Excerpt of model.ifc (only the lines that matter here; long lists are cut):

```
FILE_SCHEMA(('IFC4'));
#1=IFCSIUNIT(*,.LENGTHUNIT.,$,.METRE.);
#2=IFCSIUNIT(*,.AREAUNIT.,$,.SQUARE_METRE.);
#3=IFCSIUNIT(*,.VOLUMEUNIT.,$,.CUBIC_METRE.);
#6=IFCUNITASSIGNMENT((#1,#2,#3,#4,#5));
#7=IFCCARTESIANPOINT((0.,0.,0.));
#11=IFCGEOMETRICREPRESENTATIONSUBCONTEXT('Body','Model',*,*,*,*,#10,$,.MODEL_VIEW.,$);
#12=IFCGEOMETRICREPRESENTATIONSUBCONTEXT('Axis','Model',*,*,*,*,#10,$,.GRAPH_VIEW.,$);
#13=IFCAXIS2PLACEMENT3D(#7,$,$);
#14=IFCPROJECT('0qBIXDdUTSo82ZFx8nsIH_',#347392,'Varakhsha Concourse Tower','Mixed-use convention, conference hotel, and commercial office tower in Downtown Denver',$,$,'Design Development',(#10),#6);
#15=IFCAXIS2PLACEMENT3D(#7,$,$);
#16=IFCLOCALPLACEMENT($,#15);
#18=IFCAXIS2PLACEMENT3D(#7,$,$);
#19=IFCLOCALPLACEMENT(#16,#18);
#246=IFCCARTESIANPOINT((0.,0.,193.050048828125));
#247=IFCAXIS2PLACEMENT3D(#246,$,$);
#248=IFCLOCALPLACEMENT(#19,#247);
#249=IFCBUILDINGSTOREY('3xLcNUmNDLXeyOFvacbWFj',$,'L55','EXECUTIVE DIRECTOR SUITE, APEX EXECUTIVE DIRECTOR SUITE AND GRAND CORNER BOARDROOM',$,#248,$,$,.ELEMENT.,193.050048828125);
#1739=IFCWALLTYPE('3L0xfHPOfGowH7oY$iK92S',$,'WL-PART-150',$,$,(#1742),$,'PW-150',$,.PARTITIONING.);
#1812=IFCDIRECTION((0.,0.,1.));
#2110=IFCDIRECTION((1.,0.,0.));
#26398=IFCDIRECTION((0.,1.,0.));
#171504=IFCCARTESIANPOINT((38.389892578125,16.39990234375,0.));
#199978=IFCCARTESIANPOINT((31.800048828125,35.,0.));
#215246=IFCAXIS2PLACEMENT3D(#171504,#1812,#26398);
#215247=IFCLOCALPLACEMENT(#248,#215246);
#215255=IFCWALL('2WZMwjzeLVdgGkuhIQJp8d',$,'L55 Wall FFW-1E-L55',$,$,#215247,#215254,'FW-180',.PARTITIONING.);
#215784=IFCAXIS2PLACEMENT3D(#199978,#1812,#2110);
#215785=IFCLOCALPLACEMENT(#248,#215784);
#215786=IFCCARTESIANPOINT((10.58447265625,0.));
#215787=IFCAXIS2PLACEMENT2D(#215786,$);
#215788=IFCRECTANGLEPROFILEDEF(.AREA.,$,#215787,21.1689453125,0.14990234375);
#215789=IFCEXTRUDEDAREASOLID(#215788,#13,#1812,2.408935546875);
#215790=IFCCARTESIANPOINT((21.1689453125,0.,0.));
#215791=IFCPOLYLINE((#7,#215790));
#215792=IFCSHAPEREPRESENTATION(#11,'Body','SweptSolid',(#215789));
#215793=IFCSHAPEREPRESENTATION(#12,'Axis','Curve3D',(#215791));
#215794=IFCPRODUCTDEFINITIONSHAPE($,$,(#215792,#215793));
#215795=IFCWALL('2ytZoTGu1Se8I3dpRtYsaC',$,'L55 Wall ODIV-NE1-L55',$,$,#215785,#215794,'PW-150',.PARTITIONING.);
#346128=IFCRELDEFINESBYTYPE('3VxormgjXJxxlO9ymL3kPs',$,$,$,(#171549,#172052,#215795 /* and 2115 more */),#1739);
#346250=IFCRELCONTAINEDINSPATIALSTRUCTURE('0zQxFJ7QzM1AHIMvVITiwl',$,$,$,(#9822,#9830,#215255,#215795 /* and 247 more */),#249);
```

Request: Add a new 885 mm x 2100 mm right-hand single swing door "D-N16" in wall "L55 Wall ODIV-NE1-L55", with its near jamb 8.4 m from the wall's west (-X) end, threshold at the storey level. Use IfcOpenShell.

```python
import numpy as np
import ifcopenshell
import ifcopenshell.api.feature
import ifcopenshell.api.geometry
import ifcopenshell.api.root
import ifcopenshell.api.spatial
import ifcopenshell.geom
import ifcopenshell.util.element
import ifcopenshell.util.placement
import ifcopenshell.util.representation
import ifcopenshell.util.shape
import ifcopenshell.util.unit

model = ifcopenshell.open("model.ifc")
unit_scale = ifcopenshell.util.unit.calculate_unit_scale(model)
settings = ifcopenshell.geom.settings()


def volume(element):
    """Net volume in cubic metres, openings subtracted."""
    shape = ifcopenshell.geom.create_shape(settings, element)
    return ifcopenshell.util.shape.get_volume(shape.geometry)


wall = model.by_id(215795)
storey = ifcopenshell.util.element.get_container(wall, ifc_class="IfcBuildingStorey")
context = ifcopenshell.util.representation.get_context(model, "Model", "Body", "MODEL_VIEW")
before = volume(wall)

width, height, from_end, sill = 0.885, 2.1, 8.4, 0.0  # metres

# The wall runs along its own X axis, and the end named is its -X end.
wall_shape = ifcopenshell.geom.create_shape(settings, wall)
x, y, z = ifcopenshell.util.shape.get_vertices(wall_shape.geometry).T
start = x.min() + from_end
face, thickness = float(y.min()), float(y.max() - y.min())
wall_matrix = ifcopenshell.util.placement.get_local_placement(wall.ObjectPlacement)
level = ifcopenshell.util.placement.get_local_placement(storey.ObjectPlacement)[2, 3]


def in_wall(x, y):
    """Placement at x, y metres in the wall's axes, at sill height."""
    matrix = wall_matrix.copy()
    matrix[:, 3] = wall_matrix @ np.array([x / unit_scale, y / unit_scale, 0.0, 1.0])
    matrix[2, 3] = level + sill / unit_scale
    return matrix


# Opening: a box that overshoots both wall faces by 50 mm.
opening = ifcopenshell.api.root.create_entity(model, ifc_class="IfcOpeningElement", predefined_type="OPENING")
box = ifcopenshell.api.geometry.add_wall_representation(
    model, context=context, length=width, height=height, thickness=thickness + 0.1
)
ifcopenshell.api.geometry.assign_representation(model, product=opening, representation=box)
ifcopenshell.api.geometry.edit_object_placement(model, product=opening, matrix=in_wall(start, face - 0.05), is_si=False)
ifcopenshell.api.feature.add_feature(model, feature=opening, element=wall)

door = ifcopenshell.api.root.create_entity(model, ifc_class="IfcDoor", name="D-N16", predefined_type="DOOR")
door.OverallWidth, door.OverallHeight = width / unit_scale, height / unit_scale
door.OperationType = "SINGLE_SWING_RIGHT"
body = ifcopenshell.api.geometry.add_door_representation(
    model,
    context=context,
    overall_width=door.OverallWidth,
    overall_height=door.OverallHeight,
    operation_type="SINGLE_SWING_RIGHT",
    lining_properties={"LiningDepth": thickness / unit_scale, "ThresholdDepth": thickness / unit_scale},
)
ifcopenshell.api.geometry.assign_representation(model, product=door, representation=body)
ifcopenshell.api.spatial.assign_container(model, products=[door], relating_structure=storey)
ifcopenshell.api.feature.add_filling(model, opening=opening, element=door)

# The lining spans the wall, so the door starts at the wall face.
ifcopenshell.api.geometry.edit_object_placement(model, product=door, matrix=in_wall(start, face), is_si=False)

after = volume(wall)

print(f"wall volume {before:.3f} -> {after:.3f} m3")

model.write("model-out.ifc")
```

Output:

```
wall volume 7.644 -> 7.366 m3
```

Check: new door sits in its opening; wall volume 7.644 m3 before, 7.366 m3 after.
